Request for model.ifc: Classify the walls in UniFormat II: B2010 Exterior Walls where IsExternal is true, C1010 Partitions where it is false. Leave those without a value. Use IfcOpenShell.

First a look at what the model holds.

```python
import ifcopenshell
import ifcopenshell.util.element

model = ifcopenshell.open("model.ifc")
print(model.schema)
print("classifications:", [c.Name for c in model.by_type("IfcClassification")])
values = [ifcopenshell.util.element.get_pset(e, "Pset_WallCommon", "IsExternal") for e in model.by_type("IfcWall")]
for value in (True, False, None):
    print("IsExternal", value, values.count(value))
```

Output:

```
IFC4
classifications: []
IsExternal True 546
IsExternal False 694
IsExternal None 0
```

```python
import ifcopenshell
import ifcopenshell.api.classification
import ifcopenshell.util.element

model = ifcopenshell.open("model.ifc")

system = ifcopenshell.api.classification.add_classification(model, classification="UniFormat II")

walls = model.by_type("IfcWall")
external = {e: ifcopenshell.util.element.get_pset(e, "Pset_WallCommon", "IsExternal") for e in walls}
for flag, code, name in ((True, "B2010", "Exterior Walls"), (False, "C1010", "Partitions")):
    products = [e for e in walls if external[e] is flag]
    ifcopenshell.api.classification.add_reference(
        model, products=products, classification=system, identification=code, name=name
    )
    print(code, len(products))

model.write("model_edited.ifc")
```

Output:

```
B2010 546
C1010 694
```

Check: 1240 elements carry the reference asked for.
